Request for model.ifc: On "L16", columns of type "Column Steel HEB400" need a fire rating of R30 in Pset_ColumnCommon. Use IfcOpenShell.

First a look at what the model holds.

```python
import ifcopenshell
import ifcopenshell.util.element

model = ifcopenshell.open("model.ifc")
print(model.schema)
storey = next(s for s in model.by_type("IfcBuildingStorey") if s.Name == "L16")
columns = [e for e in ifcopenshell.util.element.get_decomposition(storey) if e.is_a("IfcColumn")]
seen = {}
for e in columns:
    element_type = ifcopenshell.util.element.get_type(e)
    key = (element_type.Name if element_type != e and element_type else None, ifcopenshell.util.element.get_pset(e, "Pset_ColumnCommon", "FireRating"))
    seen[key] = seen.get(key, 0) + 1
for (name, value), count in sorted(seen.items(), key=str):
    print(count, "x", name, "|", value)
```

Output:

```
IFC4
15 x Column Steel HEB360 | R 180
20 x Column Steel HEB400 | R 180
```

```python
import ifcopenshell
import ifcopenshell.api.pset
import ifcopenshell.util.element

model = ifcopenshell.open("model.ifc")

storey = next(s for s in model.by_type("IfcBuildingStorey") if s.Name == "L16")
columns = [e for e in ifcopenshell.util.element.get_decomposition(storey) if e.is_a("IfcColumn")]

count = 0
for e in columns:
    element_type = ifcopenshell.util.element.get_type(e)
    if element_type in (None, e) or element_type.Name != "Column Steel HEB400":
        continue
    # add_pset returns the element's existing set when there is one.
    pset = ifcopenshell.api.pset.add_pset(model, product=e, name="Pset_ColumnCommon")
    ifcopenshell.api.pset.edit_pset(model, pset=pset, properties={"FireRating": "R30"})
    count += 1

print(count, "columns updated")

model.write("model_rev.ifc")
```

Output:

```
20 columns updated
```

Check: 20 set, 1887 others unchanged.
